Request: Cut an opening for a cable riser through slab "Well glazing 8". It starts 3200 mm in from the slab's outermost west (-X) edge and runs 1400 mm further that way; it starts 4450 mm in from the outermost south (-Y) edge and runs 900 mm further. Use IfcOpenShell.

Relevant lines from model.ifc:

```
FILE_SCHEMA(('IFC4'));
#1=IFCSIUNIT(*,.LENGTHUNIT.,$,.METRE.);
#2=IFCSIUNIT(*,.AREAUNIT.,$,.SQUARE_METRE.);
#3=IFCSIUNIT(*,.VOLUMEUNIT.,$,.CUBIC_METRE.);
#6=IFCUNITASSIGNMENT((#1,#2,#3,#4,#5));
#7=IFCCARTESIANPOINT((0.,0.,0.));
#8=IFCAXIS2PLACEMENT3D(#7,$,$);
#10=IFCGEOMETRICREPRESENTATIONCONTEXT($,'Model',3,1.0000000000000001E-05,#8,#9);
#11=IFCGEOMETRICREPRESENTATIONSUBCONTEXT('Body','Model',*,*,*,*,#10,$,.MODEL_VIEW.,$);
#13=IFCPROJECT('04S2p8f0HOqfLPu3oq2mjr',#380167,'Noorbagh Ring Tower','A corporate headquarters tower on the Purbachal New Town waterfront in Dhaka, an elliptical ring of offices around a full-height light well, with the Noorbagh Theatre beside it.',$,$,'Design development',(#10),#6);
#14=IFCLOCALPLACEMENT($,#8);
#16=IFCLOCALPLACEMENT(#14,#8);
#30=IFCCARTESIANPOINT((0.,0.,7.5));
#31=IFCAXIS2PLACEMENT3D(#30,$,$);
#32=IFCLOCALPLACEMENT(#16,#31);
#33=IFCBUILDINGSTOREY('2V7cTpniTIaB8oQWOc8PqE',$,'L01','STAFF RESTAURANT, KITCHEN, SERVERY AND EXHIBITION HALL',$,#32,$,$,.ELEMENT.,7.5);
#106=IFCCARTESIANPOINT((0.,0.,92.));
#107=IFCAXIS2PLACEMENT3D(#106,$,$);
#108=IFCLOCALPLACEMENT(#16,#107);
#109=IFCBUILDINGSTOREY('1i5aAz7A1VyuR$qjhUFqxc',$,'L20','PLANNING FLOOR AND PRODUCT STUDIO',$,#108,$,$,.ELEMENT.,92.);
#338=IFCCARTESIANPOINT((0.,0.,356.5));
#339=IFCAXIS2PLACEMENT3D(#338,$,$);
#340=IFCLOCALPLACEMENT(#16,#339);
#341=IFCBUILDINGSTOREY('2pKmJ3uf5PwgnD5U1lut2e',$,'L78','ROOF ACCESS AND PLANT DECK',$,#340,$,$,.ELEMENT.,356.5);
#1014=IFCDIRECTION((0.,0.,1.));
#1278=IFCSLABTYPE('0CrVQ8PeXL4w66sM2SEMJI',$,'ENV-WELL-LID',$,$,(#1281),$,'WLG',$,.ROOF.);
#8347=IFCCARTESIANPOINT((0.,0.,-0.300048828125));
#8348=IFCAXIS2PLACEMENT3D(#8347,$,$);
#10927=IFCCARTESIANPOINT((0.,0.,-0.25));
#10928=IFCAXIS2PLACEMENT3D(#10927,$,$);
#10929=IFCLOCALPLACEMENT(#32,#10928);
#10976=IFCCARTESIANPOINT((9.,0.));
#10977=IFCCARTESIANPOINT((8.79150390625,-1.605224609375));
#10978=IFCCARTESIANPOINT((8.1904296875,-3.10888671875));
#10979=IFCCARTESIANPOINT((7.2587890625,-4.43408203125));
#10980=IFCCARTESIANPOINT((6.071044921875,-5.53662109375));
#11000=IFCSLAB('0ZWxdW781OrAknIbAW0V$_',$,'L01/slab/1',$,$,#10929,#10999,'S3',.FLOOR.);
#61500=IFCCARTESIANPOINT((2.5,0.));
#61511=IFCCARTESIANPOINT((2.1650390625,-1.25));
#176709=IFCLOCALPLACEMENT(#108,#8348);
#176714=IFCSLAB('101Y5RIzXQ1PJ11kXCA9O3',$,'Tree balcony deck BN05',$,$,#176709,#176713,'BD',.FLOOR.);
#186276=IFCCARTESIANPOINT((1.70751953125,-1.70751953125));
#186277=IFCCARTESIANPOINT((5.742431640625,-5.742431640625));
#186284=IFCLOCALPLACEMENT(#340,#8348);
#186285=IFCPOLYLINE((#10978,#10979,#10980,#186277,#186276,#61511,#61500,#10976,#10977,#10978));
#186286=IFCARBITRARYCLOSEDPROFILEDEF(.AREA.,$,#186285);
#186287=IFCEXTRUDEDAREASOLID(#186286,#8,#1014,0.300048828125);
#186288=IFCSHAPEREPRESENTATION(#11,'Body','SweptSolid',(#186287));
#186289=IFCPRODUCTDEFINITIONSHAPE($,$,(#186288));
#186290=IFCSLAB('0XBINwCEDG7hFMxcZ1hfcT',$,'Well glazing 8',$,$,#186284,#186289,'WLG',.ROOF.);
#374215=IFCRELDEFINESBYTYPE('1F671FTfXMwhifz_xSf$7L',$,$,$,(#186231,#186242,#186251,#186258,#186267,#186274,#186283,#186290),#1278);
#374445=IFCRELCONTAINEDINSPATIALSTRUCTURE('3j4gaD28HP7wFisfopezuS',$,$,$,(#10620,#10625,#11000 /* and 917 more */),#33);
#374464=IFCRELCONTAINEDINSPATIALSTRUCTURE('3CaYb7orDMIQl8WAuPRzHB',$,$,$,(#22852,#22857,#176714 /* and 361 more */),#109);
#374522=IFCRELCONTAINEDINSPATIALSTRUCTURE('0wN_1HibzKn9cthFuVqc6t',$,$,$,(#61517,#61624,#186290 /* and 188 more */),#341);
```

```python
import numpy as np
import ifcopenshell
import ifcopenshell.api.feature
import ifcopenshell.api.geometry
import ifcopenshell.api.root
import ifcopenshell.geom
import ifcopenshell.util.placement
import ifcopenshell.util.representation
import ifcopenshell.util.shape
import ifcopenshell.util.unit

model = ifcopenshell.open("model.ifc")
unit_scale = ifcopenshell.util.unit.calculate_unit_scale(model)
settings = ifcopenshell.geom.settings()


def volume(element):
    """Net volume in cubic metres, openings subtracted."""
    shape = ifcopenshell.geom.create_shape(settings, element)
    return ifcopenshell.util.shape.get_volume(shape.geometry)


slab = model.by_guid("0XBINwCEDG7hFMxcZ1hfcT")
before = volume(slab)

# Extent in the slab's own axes, in metres. The edges named are its -X and -Y sides.
slab_shape = ifcopenshell.geom.create_shape(settings, slab)
vertices = ifcopenshell.util.shape.get_vertices(slab_shape.geometry)
x_min, y_min, bottom = vertices.min(axis=0)
top = vertices[:, 2].max()

opening = ifcopenshell.api.root.create_entity(model, ifc_class="IfcOpeningElement", name="Cable riser opening", predefined_type="OPENING")
context = ifcopenshell.util.representation.get_context(model, "Model", "Body", "MODEL_VIEW")
width, depth = 1.4, 0.9
outline = [(0.0, 0.0), (width, 0.0), (width, depth), (0.0, depth), (0.0, 0.0)]
# Overshoot both faces by 50 mm so the cut is clean.
shape = ifcopenshell.api.geometry.add_slab_representation(
    model, context=context, depth=top - bottom + 0.1, polyline=outline
)
ifcopenshell.api.geometry.assign_representation(model, product=opening, representation=shape)

matrix = ifcopenshell.util.placement.get_local_placement(slab.ObjectPlacement)
matrix[:, 3] = matrix @ np.append(np.array([x_min + 3.2, y_min + 4.45, bottom - 0.05]) / unit_scale, 1.0)
ifcopenshell.api.geometry.edit_object_placement(model, product=opening, matrix=matrix, is_si=False)
ifcopenshell.api.feature.add_feature(model, feature=opening, element=slab)

after = volume(slab)

print(f"slab volume {before:.3f} -> {after:.3f} m3")

model.write("model_v2.ifc")
```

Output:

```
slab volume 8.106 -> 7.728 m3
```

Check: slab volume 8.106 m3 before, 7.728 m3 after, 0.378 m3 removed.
